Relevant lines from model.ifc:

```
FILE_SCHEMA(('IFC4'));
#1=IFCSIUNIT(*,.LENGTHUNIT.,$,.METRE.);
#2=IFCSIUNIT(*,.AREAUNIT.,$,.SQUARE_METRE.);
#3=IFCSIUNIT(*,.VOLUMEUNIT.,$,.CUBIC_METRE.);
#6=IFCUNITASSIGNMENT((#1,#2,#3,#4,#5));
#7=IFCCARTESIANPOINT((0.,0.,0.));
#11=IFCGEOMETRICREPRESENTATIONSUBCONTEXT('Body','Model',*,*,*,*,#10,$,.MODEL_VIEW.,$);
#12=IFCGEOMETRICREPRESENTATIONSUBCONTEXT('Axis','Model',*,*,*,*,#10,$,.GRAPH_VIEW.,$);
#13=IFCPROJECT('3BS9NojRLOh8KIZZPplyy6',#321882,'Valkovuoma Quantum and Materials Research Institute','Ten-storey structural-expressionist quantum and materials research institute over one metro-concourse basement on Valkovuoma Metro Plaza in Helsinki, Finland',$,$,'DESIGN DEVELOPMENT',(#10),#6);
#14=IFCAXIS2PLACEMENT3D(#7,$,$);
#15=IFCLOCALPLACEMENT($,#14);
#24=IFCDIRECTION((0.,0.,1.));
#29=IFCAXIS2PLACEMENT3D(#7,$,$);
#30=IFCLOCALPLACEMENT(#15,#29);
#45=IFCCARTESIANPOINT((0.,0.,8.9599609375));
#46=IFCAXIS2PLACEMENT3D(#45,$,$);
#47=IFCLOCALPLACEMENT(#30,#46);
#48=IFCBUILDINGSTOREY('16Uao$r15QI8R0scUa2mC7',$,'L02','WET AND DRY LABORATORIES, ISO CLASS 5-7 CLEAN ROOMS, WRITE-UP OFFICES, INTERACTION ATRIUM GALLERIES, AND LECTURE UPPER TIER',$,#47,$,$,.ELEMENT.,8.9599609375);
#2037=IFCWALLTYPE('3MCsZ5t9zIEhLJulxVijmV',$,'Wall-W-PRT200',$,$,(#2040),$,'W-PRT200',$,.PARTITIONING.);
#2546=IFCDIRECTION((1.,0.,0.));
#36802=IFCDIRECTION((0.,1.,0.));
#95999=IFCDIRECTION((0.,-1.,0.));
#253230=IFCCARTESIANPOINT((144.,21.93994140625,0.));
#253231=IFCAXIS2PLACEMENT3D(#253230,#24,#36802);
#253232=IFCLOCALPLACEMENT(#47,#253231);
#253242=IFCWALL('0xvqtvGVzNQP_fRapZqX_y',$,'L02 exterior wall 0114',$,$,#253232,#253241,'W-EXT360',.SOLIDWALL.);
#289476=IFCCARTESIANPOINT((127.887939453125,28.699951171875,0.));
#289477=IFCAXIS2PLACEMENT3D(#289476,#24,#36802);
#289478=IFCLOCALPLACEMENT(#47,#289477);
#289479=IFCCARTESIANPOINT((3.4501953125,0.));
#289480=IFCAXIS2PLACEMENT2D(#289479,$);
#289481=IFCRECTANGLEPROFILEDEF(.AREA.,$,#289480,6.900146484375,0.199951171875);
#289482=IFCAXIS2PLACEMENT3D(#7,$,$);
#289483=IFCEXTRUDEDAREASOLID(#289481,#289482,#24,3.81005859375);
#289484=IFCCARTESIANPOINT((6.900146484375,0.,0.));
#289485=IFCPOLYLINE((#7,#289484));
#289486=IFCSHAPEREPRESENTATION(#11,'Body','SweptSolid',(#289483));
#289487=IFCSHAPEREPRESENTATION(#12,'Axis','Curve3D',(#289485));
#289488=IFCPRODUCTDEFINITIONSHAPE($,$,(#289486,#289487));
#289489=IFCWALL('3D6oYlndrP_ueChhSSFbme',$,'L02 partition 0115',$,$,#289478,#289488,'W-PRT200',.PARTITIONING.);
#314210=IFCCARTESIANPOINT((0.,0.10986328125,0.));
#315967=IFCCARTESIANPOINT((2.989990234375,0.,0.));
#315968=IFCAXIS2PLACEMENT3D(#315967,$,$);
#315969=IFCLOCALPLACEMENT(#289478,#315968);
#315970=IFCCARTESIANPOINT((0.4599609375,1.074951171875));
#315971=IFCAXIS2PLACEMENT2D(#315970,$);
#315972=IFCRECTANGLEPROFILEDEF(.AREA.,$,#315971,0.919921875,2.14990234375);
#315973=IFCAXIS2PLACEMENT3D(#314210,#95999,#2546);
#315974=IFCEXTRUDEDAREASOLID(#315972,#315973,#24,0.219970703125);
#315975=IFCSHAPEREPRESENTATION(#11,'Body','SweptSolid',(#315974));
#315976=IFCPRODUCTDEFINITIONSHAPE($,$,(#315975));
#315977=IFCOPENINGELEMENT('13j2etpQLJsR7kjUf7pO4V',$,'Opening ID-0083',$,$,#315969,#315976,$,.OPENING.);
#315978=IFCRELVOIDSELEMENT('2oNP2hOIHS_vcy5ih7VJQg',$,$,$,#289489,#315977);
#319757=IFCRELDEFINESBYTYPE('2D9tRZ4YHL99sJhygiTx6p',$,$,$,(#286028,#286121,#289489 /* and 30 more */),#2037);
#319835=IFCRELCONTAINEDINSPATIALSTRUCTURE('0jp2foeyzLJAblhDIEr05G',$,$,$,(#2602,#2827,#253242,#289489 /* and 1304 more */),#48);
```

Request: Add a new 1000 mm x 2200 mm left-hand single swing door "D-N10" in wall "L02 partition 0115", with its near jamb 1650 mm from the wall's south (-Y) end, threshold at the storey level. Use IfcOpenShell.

```python
import numpy as np
import ifcopenshell
import ifcopenshell.api.feature
import ifcopenshell.api.geometry
import ifcopenshell.api.root
import ifcopenshell.api.spatial
import ifcopenshell.geom
import ifcopenshell.util.element
import ifcopenshell.util.placement
import ifcopenshell.util.representation
import ifcopenshell.util.shape
import ifcopenshell.util.unit

model = ifcopenshell.open("model.ifc")
unit_scale = ifcopenshell.util.unit.calculate_unit_scale(model)
settings = ifcopenshell.geom.settings()


def volume(element):
    """Net volume in cubic metres, openings subtracted."""
    shape = ifcopenshell.geom.create_shape(settings, element)
    return ifcopenshell.util.shape.get_volume(shape.geometry)


wall = model.by_guid("3D6oYlndrP_ueChhSSFbme")
storey = ifcopenshell.util.element.get_container(wall, ifc_class="IfcBuildingStorey")
context = ifcopenshell.util.representation.get_context(model, "Model", "Body", "MODEL_VIEW")
before = volume(wall)

width, height, from_end, sill = 1, 2.2, 1.65, 0.0  # metres

# The wall runs along its own X axis, and the end named is its -X end.
wall_shape = ifcopenshell.geom.create_shape(settings, wall)
x, y, z = ifcopenshell.util.shape.get_vertices(wall_shape.geometry).T
start = x.min() + from_end
face, thickness = float(y.min()), float(y.max() - y.min())
wall_matrix = ifcopenshell.util.placement.get_local_placement(wall.ObjectPlacement)
level = ifcopenshell.util.placement.get_local_placement(storey.ObjectPlacement)[2, 3]


def in_wall(x, y):
    """Placement at x, y metres in the wall's axes, at sill height."""
    matrix = wall_matrix.copy()
    matrix[:, 3] = wall_matrix @ np.array([x / unit_scale, y / unit_scale, 0.0, 1.0])
    matrix[2, 3] = level + sill / unit_scale
    return matrix


# Opening: a box that overshoots both wall faces by 50 mm.
opening = ifcopenshell.api.root.create_entity(model, ifc_class="IfcOpeningElement", predefined_type="OPENING")
box = ifcopenshell.api.geometry.add_wall_representation(
    model, context=context, length=width, height=height, thickness=thickness + 0.1
)
ifcopenshell.api.geometry.assign_representation(model, product=opening, representation=box)
ifcopenshell.api.geometry.edit_object_placement(model, product=opening, matrix=in_wall(start, face - 0.05), is_si=False)
ifcopenshell.api.feature.add_feature(model, feature=opening, element=wall)

door = ifcopenshell.api.root.create_entity(model, ifc_class="IfcDoor", name="D-N10", predefined_type="DOOR")
door.OverallWidth, door.OverallHeight = width / unit_scale, height / unit_scale
door.OperationType = "SINGLE_SWING_LEFT"
body = ifcopenshell.api.geometry.add_door_representation(
    model,
    context=context,
    overall_width=door.OverallWidth,
    overall_height=door.OverallHeight,
    operation_type="SINGLE_SWING_LEFT",
    lining_properties={"LiningDepth": thickness / unit_scale, "ThresholdDepth": thickness / unit_scale},
)
ifcopenshell.api.geometry.assign_representation(model, product=door, representation=body)
ifcopenshell.api.spatial.assign_container(model, products=[door], relating_structure=storey)
ifcopenshell.api.feature.add_filling(model, opening=opening, element=door)

# The lining spans the wall, so the door starts at the wall face.
ifcopenshell.api.geometry.edit_object_placement(model, product=door, matrix=in_wall(start, face), is_si=False)

after = volume(wall)

print(f"wall volume {before:.3f} -> {after:.3f} m3")

model.write("model_updated.ifc")
```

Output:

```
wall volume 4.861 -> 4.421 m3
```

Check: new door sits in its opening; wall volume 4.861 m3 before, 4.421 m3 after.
